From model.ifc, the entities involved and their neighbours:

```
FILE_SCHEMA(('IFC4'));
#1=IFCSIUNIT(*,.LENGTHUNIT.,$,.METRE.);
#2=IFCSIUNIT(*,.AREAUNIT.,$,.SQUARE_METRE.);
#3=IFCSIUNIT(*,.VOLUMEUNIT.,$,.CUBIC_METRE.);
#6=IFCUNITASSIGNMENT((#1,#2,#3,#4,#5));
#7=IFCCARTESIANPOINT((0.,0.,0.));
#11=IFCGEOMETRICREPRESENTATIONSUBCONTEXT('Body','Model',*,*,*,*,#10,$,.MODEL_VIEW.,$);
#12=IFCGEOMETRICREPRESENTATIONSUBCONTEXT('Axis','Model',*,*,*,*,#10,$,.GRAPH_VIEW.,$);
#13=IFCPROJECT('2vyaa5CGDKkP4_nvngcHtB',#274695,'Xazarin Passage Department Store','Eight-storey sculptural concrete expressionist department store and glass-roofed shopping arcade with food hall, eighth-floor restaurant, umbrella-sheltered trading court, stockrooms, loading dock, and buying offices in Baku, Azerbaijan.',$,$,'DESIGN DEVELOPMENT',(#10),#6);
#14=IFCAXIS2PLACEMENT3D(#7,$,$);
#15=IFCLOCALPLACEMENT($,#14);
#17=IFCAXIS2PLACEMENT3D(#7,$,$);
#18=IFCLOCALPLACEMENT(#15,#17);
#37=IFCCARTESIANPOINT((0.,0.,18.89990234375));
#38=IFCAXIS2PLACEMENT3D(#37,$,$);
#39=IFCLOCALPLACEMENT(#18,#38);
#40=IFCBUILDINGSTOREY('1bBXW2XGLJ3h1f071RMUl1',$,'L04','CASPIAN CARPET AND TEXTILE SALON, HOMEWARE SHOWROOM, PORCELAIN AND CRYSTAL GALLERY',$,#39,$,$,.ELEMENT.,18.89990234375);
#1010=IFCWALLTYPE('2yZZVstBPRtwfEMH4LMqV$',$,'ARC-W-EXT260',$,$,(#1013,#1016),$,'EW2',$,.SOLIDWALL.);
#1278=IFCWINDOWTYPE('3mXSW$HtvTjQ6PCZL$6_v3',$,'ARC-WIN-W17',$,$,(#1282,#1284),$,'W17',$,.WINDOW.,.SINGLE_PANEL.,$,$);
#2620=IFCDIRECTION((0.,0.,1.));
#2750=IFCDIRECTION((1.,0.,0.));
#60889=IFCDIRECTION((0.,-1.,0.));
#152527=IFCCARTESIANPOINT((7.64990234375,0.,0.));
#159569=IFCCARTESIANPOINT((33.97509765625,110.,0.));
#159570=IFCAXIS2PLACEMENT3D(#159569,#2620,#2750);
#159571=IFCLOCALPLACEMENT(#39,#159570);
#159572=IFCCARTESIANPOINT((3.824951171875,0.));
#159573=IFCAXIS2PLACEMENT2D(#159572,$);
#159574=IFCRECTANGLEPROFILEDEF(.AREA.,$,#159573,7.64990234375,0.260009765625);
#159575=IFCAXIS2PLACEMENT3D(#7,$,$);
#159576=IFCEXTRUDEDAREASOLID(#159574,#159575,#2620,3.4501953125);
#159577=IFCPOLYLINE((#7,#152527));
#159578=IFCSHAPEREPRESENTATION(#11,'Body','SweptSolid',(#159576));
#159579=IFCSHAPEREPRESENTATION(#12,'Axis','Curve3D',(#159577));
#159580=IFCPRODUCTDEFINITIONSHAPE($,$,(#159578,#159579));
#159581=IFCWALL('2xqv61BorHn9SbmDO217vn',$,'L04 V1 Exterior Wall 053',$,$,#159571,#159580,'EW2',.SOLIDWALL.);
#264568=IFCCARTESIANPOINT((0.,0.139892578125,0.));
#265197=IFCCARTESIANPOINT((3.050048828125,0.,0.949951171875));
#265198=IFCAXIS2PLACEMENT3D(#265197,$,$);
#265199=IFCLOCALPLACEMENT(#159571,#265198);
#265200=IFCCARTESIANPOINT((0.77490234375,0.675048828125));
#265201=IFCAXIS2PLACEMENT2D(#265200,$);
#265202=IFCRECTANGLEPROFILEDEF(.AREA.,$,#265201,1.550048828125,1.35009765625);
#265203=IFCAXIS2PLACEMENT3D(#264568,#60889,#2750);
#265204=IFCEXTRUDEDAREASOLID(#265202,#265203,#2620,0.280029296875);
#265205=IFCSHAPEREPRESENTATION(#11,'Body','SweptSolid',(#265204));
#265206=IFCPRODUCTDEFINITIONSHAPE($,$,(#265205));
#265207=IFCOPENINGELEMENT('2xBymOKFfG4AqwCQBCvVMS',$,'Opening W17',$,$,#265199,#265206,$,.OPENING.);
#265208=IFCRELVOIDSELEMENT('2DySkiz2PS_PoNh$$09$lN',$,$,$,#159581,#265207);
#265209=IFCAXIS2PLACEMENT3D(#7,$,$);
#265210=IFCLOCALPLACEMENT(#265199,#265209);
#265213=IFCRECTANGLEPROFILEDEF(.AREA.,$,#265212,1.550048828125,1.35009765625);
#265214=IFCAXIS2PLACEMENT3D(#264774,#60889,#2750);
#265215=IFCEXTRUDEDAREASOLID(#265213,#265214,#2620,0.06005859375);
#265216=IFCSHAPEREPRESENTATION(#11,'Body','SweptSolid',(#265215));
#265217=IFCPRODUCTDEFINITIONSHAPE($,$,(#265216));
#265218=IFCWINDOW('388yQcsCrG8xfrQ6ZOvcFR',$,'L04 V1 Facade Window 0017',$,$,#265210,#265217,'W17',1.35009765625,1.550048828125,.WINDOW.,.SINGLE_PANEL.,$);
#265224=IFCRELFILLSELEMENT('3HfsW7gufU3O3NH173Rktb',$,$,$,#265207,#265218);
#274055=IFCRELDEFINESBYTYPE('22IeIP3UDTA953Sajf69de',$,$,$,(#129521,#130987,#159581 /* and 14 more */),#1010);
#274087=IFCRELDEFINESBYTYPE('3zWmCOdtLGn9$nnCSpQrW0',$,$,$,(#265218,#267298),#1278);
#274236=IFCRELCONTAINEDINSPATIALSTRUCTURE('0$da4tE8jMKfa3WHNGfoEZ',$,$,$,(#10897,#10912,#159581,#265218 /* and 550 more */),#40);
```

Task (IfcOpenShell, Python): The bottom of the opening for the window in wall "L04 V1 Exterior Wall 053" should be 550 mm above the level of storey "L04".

```python
import numpy as np
import ifcopenshell
import ifcopenshell.api.geometry
import ifcopenshell.geom
import ifcopenshell.util.element
import ifcopenshell.util.placement
import ifcopenshell.util.shape
import ifcopenshell.util.unit

model = ifcopenshell.open("model.ifc")
unit_scale = ifcopenshell.util.unit.calculate_unit_scale(model)

window = model.by_id(265218)
opening = window.FillsVoids[0].RelatingOpeningElement
storey = ifcopenshell.util.element.get_container(window, ifc_class="IfcBuildingStorey")
level = ifcopenshell.util.placement.get_local_placement(storey.ObjectPlacement)[2, 3]

# The opening's origin need not be at the sill, so measure its lowest point.
shape = ifcopenshell.geom.create_shape(ifcopenshell.geom.settings(), opening)
bottom = ifcopenshell.util.shape.get_shape_bottom_elevation(shape, shape.geometry) / unit_scale
dz = level + 0.55 - bottom

shift = np.array([0.0, 0.0, dz])
# The window is placed relative to its opening, so it follows when the opening moves.
matrix = ifcopenshell.util.placement.get_local_placement(opening.ObjectPlacement)
matrix[:3, 3] += shift
ifcopenshell.api.geometry.edit_object_placement(
    model, product=opening, matrix=matrix, is_si=False, should_transform_children=True
)

print(f"moved by {dz * unit_scale:+.3f} m")

model.write("model_rev.ifc")
```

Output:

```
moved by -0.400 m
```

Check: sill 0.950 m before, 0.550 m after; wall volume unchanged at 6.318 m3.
